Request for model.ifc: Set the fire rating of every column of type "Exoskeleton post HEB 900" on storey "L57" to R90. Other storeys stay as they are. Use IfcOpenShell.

First a look at what the model holds.

```python
import ifcopenshell
import ifcopenshell.util.element

model = ifcopenshell.open("model.ifc")
print(model.schema)
storey = next(s for s in model.by_type("IfcBuildingStorey") if s.Name == "L57")
columns = [e for e in ifcopenshell.util.element.get_decomposition(storey) if e.is_a("IfcColumn")]
seen = {}
for e in columns:
    element_type = ifcopenshell.util.element.get_type(e)
    key = (element_type.Name if element_type != e and element_type else None, ifcopenshell.util.element.get_pset(e, "Pset_ColumnCommon", "FireRating"))
    seen[key] = seen.get(key, 0) + 1
for (name, value), count in sorted(seen.items(), key=str):
    print(count, "x", name, "|", value)
```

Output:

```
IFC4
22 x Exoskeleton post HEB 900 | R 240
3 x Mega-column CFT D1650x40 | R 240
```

```python
import ifcopenshell
import ifcopenshell.api.pset
import ifcopenshell.util.element

model = ifcopenshell.open("model.ifc")

storey = next(s for s in model.by_type("IfcBuildingStorey") if s.Name == "L57")
columns = [e for e in ifcopenshell.util.element.get_decomposition(storey) if e.is_a("IfcColumn")]

count = 0
for e in columns:
    element_type = ifcopenshell.util.element.get_type(e)
    if element_type in (None, e) or element_type.Name != "Exoskeleton post HEB 900":
        continue
    found = ifcopenshell.util.element.get_pset(e, "Pset_ColumnCommon", should_inherit=False)
    if found:
        pset = model.by_id(found["id"])
        if len(ifcopenshell.util.element.get_elements_by_pset(pset)) > 1:
            pset = ifcopenshell.api.pset.unshare_pset(model, products=[e], pset=pset)[0]
    else:
        pset = ifcopenshell.api.pset.add_pset(model, product=e, name="Pset_ColumnCommon")
    ifcopenshell.api.pset.edit_pset(model, pset=pset, properties={"FireRating": "R90"})
    count += 1

print(count, "columns updated")

model.write("model_edited.ifc")
```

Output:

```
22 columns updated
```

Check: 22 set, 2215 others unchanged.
